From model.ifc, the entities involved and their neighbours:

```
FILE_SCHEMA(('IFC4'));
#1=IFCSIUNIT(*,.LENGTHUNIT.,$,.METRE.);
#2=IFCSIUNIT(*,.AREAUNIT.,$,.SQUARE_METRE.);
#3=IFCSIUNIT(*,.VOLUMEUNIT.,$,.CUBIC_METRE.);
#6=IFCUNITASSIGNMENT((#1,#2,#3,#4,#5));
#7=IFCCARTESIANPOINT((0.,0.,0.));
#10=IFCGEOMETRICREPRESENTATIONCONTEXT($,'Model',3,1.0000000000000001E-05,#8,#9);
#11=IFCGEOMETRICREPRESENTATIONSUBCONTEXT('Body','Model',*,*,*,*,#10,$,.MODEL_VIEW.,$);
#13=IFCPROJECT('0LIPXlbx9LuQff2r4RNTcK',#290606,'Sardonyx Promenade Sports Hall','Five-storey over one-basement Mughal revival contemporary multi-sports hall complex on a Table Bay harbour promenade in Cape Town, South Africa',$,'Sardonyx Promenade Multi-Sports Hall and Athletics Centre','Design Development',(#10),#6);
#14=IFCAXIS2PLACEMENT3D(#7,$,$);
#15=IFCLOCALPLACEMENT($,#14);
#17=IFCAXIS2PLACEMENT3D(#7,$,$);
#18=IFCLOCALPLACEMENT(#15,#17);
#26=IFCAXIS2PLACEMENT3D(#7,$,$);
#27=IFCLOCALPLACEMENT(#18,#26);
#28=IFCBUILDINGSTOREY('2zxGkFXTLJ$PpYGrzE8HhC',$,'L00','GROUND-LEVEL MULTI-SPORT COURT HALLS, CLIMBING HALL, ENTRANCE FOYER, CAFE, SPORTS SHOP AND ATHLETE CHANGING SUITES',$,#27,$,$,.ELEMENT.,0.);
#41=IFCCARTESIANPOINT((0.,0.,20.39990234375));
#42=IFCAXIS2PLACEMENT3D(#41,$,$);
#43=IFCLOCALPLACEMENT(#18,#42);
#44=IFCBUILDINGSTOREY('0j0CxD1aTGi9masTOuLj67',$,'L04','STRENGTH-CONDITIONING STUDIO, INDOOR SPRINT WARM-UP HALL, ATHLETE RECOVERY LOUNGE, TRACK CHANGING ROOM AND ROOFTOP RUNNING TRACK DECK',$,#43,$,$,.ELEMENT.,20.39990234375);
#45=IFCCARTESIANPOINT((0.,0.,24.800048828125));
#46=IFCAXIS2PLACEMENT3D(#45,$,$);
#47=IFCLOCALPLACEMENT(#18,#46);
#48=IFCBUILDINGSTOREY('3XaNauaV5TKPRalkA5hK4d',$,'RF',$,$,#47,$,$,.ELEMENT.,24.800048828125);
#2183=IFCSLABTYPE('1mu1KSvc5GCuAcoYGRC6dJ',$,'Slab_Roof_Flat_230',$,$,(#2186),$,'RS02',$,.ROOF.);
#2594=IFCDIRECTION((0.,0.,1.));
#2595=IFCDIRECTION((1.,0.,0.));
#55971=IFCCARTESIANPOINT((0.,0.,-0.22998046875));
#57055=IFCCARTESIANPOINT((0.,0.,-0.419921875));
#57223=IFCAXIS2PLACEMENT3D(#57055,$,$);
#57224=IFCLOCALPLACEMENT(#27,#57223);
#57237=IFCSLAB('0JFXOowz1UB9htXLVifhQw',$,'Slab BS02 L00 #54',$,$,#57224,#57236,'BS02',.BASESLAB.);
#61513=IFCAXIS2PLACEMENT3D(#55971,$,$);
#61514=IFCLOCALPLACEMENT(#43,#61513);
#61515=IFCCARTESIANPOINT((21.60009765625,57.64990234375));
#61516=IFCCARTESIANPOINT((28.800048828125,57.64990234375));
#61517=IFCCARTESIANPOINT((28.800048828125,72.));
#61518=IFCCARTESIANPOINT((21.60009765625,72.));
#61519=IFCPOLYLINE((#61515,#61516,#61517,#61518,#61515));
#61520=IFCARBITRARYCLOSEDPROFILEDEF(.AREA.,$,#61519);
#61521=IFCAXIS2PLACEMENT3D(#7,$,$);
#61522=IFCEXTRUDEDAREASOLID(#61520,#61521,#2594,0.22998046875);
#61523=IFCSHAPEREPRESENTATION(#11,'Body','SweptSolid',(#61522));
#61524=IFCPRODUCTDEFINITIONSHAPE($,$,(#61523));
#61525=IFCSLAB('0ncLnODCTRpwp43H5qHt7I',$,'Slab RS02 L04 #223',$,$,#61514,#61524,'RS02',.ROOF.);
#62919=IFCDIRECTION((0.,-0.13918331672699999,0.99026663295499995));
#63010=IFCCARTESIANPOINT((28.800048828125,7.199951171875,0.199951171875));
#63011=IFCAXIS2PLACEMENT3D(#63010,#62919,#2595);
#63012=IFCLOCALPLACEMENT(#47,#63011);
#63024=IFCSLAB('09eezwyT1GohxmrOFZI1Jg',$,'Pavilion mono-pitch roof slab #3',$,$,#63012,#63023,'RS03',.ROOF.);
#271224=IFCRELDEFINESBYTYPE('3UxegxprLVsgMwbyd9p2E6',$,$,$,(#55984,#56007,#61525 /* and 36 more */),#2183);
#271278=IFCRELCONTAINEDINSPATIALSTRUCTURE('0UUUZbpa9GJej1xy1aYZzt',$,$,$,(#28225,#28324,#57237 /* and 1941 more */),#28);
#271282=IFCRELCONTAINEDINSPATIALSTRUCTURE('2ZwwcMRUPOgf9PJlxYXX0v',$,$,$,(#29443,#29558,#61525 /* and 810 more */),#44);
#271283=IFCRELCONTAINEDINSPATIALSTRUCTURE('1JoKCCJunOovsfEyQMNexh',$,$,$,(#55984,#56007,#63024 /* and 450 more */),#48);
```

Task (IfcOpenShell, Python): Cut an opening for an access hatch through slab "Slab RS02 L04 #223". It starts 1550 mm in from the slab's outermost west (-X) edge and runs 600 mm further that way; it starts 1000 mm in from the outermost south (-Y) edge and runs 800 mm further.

```python
import numpy as np
import ifcopenshell
import ifcopenshell.api.feature
import ifcopenshell.api.geometry
import ifcopenshell.api.root
import ifcopenshell.geom
import ifcopenshell.util.placement
import ifcopenshell.util.representation
import ifcopenshell.util.shape
import ifcopenshell.util.unit

model = ifcopenshell.open("model.ifc")
unit_scale = ifcopenshell.util.unit.calculate_unit_scale(model)
settings = ifcopenshell.geom.settings()


def volume(element):
    """Net volume in cubic metres, openings subtracted."""
    shape = ifcopenshell.geom.create_shape(settings, element)
    return ifcopenshell.util.shape.get_volume(shape.geometry)


slab = model.by_id(61525)
before = volume(slab)

# Extent in the slab's own axes, in metres. The edges named are its -X and -Y sides.
slab_shape = ifcopenshell.geom.create_shape(settings, slab)
vertices = ifcopenshell.util.shape.get_vertices(slab_shape.geometry)
x_min, y_min, bottom = vertices.min(axis=0)
top = vertices[:, 2].max()

opening = ifcopenshell.api.root.create_entity(model, ifc_class="IfcOpeningElement", name="Access hatch opening", predefined_type="OPENING")
context = ifcopenshell.util.representation.get_context(model, "Model", "Body", "MODEL_VIEW")
width, depth = 0.6, 0.8
outline = [(0.0, 0.0), (width, 0.0), (width, depth), (0.0, depth), (0.0, 0.0)]
# Overshoot both faces by 50 mm so the cut is clean.
shape = ifcopenshell.api.geometry.add_slab_representation(
    model, context=context, depth=top - bottom + 0.1, polyline=outline
)
ifcopenshell.api.geometry.assign_representation(model, product=opening, representation=shape)

matrix = ifcopenshell.util.placement.get_local_placement(slab.ObjectPlacement)
matrix[:, 3] = matrix @ np.append(np.array([x_min + 1.55, y_min + 1, bottom - 0.05]) / unit_scale, 1.0)
ifcopenshell.api.geometry.edit_object_placement(model, product=opening, matrix=matrix, is_si=False)
ifcopenshell.api.feature.add_feature(model, feature=opening, element=slab)

after = volume(slab)

print(f"slab volume {before:.3f} -> {after:.3f} m3")

model.write("model_v2.ifc")
```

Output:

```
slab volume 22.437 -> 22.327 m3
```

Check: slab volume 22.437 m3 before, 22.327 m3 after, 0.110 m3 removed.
